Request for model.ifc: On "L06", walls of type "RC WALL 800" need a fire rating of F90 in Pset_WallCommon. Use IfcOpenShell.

First a look at what the model holds.

```python
import ifcopenshell
import ifcopenshell.util.element

model = ifcopenshell.open("model.ifc")
print(model.schema)
storey = next(s for s in model.by_type("IfcBuildingStorey") if s.Name == "L06")
walls = [e for e in ifcopenshell.util.element.get_decomposition(storey) if e.is_a("IfcWall")]
seen = {}
for e in walls:
    element_type = ifcopenshell.util.element.get_type(e)
    key = (element_type.Name if element_type != e and element_type else None, ifcopenshell.util.element.get_pset(e, "Pset_WallCommon", "FireRating"))
    seen[key] = seen.get(key, 0) + 1
for (name, value), count in sorted(seen.items(), key=str):
    print(count, "x", name, "|", value)
```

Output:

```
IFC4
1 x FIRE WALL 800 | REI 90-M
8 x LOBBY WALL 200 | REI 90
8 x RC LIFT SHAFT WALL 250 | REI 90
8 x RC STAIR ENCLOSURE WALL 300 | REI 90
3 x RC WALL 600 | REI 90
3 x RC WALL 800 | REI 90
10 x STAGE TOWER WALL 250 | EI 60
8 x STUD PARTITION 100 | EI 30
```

```python
import ifcopenshell
import ifcopenshell.api.pset
import ifcopenshell.util.element

model = ifcopenshell.open("model.ifc")

storey = next(s for s in model.by_type("IfcBuildingStorey") if s.Name == "L06")
walls = [e for e in ifcopenshell.util.element.get_decomposition(storey) if e.is_a("IfcWall")]

count = 0
for e in walls:
    element_type = ifcopenshell.util.element.get_type(e)
    if element_type in (None, e) or element_type.Name != "RC WALL 800":
        continue
    # add_pset returns the element's existing set when there is one.
    pset = ifcopenshell.api.pset.add_pset(model, product=e, name="Pset_WallCommon")
    ifcopenshell.api.pset.edit_pset(model, pset=pset, properties={"FireRating": "F90"})
    count += 1

print(count, "walls updated")

model.write("model_rev.ifc")
```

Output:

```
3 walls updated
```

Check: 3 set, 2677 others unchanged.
